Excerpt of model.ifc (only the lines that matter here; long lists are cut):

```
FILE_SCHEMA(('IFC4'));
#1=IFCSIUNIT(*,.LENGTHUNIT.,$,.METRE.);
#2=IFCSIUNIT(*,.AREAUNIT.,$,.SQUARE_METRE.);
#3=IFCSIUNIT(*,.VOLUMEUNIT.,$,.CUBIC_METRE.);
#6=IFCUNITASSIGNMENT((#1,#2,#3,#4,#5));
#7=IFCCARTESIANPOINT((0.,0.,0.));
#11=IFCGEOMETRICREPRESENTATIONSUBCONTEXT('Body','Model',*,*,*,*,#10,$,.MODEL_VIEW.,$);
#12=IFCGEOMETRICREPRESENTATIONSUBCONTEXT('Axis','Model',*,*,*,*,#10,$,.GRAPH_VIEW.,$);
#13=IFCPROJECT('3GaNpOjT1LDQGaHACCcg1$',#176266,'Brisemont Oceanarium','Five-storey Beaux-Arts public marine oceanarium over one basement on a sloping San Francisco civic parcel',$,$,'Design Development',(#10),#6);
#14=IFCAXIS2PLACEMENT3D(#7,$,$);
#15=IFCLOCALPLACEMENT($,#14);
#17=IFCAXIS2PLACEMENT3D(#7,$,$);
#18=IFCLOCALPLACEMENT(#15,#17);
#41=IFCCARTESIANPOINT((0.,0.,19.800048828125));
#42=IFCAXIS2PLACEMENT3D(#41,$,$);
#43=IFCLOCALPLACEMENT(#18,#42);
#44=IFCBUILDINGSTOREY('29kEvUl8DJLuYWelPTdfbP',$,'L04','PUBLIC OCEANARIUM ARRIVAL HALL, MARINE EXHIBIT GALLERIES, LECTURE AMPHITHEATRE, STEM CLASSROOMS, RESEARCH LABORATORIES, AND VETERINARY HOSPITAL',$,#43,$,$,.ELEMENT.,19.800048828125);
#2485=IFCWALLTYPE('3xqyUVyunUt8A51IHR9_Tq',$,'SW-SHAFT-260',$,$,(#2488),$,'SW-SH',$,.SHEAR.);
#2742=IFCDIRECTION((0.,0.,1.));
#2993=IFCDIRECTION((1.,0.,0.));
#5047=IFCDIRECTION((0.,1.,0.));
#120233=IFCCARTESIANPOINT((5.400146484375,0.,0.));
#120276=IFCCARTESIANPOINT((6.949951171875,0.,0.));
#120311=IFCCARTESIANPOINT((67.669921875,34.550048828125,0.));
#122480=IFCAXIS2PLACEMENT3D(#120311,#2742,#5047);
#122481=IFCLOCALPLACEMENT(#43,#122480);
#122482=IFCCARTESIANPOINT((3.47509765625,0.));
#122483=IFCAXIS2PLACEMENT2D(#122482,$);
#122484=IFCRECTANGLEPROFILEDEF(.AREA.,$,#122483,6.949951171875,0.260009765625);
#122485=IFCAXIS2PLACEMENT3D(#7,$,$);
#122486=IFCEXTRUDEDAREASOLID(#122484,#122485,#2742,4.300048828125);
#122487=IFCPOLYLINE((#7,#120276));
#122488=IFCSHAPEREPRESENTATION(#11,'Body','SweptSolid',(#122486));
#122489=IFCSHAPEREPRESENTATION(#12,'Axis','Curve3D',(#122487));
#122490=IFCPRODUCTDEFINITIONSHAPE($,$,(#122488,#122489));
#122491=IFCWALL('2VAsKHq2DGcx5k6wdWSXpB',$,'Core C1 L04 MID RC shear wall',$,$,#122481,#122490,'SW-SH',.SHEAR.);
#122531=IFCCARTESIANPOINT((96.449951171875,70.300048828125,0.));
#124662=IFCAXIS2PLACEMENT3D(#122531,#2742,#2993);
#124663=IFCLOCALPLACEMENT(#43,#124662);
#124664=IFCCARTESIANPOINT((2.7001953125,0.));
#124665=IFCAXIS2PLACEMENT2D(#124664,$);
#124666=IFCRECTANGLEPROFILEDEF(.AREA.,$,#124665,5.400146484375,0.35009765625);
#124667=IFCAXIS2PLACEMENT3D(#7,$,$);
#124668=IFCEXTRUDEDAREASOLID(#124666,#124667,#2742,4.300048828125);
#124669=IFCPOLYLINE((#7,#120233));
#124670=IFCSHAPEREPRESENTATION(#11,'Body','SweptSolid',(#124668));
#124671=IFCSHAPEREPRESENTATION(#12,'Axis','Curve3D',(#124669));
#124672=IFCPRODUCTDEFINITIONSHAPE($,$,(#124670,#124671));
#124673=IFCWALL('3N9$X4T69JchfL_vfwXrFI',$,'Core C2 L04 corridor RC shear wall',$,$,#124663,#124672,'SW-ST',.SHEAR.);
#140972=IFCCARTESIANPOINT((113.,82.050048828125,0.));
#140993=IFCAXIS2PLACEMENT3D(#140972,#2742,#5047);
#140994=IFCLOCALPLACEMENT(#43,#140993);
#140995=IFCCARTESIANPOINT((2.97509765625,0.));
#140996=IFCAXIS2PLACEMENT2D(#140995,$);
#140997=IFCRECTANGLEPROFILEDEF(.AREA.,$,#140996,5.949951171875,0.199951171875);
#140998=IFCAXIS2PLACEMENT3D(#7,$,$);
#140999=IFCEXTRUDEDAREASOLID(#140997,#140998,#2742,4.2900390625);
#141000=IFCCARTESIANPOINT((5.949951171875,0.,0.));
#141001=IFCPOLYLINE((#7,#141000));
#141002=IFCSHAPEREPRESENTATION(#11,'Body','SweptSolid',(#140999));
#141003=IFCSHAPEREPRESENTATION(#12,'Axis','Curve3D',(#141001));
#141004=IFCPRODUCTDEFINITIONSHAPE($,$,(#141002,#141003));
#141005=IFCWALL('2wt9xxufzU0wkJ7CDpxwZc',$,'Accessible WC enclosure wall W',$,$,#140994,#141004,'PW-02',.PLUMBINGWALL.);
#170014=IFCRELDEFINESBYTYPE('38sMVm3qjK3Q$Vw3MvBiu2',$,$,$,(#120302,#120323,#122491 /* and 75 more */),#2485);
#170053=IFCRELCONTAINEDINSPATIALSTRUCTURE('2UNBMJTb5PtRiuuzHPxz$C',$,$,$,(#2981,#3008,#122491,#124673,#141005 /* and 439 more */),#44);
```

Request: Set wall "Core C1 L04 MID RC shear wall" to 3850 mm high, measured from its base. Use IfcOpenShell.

```python
import ifcopenshell
import ifcopenshell.geom
import ifcopenshell.util.representation
import ifcopenshell.util.shape
import ifcopenshell.util.unit

model = ifcopenshell.open("model.ifc")
unit_scale = ifcopenshell.util.unit.calculate_unit_scale(model)
settings = ifcopenshell.geom.settings()


def volume(element):
    """Net volume in cubic metres, openings subtracted."""
    shape = ifcopenshell.geom.create_shape(settings, element)
    return ifcopenshell.util.shape.get_volume(shape.geometry)


wall = model.by_guid("2VAsKHq2DGcx5k6wdWSXpB")
before = volume(wall)

body = ifcopenshell.util.representation.get_representation(wall, "Model", "Body")
solid = body.Items[0]
old_height = solid.Depth
solid.Depth = 3.85 / unit_scale
after = volume(wall)

print(f"height {old_height:g} -> {solid.Depth:g}, volume {before:.3f} -> {after:.3f} m3")

model.write("model_updated.ifc")
```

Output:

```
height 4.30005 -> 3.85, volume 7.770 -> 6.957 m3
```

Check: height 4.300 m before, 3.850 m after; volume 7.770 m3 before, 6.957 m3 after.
